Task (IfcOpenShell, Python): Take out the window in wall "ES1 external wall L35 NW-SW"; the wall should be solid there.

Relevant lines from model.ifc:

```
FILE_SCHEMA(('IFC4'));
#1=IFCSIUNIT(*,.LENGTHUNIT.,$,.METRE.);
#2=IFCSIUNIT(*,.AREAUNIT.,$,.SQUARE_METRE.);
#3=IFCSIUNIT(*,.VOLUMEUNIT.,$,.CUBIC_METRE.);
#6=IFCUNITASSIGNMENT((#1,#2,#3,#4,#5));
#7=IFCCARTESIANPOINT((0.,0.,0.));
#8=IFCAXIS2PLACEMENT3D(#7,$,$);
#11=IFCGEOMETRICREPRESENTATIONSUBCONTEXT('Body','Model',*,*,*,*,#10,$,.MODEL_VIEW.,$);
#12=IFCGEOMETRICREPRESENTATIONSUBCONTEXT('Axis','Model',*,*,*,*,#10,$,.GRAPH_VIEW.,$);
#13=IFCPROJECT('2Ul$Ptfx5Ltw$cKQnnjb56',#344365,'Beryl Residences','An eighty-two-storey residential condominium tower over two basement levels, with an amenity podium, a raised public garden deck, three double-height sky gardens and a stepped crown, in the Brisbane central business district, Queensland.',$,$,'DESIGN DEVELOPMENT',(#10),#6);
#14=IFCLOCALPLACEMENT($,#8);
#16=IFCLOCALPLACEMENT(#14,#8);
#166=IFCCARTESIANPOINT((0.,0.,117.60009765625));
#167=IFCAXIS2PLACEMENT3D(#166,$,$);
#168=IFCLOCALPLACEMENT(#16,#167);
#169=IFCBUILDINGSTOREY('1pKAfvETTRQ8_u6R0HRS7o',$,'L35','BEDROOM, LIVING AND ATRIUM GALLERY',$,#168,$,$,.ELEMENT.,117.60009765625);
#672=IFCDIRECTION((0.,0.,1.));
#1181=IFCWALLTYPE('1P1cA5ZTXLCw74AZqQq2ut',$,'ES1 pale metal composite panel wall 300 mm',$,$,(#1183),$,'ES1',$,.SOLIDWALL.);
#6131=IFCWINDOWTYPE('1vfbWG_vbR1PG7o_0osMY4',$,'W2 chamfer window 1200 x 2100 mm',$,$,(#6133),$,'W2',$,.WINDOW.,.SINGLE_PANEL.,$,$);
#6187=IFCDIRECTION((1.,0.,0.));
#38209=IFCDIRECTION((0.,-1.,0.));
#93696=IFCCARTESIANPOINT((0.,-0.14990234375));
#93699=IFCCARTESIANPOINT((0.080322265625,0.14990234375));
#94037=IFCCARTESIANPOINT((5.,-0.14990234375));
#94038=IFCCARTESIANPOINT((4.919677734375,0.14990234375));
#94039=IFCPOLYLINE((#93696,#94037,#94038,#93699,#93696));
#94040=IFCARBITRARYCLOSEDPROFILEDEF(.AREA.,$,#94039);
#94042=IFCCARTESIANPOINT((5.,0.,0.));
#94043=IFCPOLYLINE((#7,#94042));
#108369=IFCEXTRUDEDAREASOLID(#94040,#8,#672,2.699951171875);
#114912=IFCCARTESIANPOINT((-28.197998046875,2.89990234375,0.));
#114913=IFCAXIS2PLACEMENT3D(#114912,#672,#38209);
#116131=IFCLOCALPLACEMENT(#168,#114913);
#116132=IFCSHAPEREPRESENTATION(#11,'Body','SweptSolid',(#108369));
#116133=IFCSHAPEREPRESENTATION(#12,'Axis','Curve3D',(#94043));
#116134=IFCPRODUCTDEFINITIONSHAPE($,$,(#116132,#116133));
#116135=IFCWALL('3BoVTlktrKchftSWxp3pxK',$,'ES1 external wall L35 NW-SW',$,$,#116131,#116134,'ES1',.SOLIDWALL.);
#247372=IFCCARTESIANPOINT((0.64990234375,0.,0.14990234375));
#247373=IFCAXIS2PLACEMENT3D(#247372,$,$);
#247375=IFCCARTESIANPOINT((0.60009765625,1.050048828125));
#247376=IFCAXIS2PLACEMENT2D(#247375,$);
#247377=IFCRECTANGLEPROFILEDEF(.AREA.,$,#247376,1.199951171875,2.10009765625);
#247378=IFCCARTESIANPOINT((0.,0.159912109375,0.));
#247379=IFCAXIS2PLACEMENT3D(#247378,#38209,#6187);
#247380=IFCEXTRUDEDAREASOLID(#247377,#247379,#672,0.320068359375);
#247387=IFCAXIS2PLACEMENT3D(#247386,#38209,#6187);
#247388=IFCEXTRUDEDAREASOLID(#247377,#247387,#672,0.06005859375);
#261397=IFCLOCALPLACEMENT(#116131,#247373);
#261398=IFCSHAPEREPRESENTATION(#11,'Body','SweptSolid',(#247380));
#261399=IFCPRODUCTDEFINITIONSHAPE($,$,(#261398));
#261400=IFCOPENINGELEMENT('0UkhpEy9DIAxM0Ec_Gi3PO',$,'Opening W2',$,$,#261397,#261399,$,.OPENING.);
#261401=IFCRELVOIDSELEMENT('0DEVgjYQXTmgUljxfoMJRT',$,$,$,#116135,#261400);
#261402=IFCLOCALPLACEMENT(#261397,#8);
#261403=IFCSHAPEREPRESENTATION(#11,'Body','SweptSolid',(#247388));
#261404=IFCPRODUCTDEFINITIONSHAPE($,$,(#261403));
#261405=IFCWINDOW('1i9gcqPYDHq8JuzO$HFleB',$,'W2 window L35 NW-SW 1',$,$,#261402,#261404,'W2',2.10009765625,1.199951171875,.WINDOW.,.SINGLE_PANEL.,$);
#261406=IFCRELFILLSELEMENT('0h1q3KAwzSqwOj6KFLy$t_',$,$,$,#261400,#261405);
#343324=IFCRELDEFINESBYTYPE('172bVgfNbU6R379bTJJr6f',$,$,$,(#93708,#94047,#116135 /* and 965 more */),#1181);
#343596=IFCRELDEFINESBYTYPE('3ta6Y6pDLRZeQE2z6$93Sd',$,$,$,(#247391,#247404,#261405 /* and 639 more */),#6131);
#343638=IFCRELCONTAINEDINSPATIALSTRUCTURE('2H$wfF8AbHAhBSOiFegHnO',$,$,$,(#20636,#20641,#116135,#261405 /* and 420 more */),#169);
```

```python
import ifcopenshell
import ifcopenshell.api.feature
import ifcopenshell.api.root
import ifcopenshell.geom
import ifcopenshell.util.shape

model = ifcopenshell.open("model.ifc")
settings = ifcopenshell.geom.settings()


def volume(element):
    """Net volume in cubic metres, openings subtracted."""
    shape = ifcopenshell.geom.create_shape(settings, element)
    return ifcopenshell.util.shape.get_volume(shape.geometry)


window = model.by_id(261405)
opening = window.FillsVoids[0].RelatingOpeningElement
wall = opening.VoidsElements[0].RelatingBuildingElement
before = volume(wall)

ifcopenshell.api.root.remove_product(model, product=window)
ifcopenshell.api.feature.remove_feature(model, feature=opening)

after = volume(wall)

print(f"wall volume {before:.3f} -> {after:.3f} m3")

model.write("model_updated.ifc")
```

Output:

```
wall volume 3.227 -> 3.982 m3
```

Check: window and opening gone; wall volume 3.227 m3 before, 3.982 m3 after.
